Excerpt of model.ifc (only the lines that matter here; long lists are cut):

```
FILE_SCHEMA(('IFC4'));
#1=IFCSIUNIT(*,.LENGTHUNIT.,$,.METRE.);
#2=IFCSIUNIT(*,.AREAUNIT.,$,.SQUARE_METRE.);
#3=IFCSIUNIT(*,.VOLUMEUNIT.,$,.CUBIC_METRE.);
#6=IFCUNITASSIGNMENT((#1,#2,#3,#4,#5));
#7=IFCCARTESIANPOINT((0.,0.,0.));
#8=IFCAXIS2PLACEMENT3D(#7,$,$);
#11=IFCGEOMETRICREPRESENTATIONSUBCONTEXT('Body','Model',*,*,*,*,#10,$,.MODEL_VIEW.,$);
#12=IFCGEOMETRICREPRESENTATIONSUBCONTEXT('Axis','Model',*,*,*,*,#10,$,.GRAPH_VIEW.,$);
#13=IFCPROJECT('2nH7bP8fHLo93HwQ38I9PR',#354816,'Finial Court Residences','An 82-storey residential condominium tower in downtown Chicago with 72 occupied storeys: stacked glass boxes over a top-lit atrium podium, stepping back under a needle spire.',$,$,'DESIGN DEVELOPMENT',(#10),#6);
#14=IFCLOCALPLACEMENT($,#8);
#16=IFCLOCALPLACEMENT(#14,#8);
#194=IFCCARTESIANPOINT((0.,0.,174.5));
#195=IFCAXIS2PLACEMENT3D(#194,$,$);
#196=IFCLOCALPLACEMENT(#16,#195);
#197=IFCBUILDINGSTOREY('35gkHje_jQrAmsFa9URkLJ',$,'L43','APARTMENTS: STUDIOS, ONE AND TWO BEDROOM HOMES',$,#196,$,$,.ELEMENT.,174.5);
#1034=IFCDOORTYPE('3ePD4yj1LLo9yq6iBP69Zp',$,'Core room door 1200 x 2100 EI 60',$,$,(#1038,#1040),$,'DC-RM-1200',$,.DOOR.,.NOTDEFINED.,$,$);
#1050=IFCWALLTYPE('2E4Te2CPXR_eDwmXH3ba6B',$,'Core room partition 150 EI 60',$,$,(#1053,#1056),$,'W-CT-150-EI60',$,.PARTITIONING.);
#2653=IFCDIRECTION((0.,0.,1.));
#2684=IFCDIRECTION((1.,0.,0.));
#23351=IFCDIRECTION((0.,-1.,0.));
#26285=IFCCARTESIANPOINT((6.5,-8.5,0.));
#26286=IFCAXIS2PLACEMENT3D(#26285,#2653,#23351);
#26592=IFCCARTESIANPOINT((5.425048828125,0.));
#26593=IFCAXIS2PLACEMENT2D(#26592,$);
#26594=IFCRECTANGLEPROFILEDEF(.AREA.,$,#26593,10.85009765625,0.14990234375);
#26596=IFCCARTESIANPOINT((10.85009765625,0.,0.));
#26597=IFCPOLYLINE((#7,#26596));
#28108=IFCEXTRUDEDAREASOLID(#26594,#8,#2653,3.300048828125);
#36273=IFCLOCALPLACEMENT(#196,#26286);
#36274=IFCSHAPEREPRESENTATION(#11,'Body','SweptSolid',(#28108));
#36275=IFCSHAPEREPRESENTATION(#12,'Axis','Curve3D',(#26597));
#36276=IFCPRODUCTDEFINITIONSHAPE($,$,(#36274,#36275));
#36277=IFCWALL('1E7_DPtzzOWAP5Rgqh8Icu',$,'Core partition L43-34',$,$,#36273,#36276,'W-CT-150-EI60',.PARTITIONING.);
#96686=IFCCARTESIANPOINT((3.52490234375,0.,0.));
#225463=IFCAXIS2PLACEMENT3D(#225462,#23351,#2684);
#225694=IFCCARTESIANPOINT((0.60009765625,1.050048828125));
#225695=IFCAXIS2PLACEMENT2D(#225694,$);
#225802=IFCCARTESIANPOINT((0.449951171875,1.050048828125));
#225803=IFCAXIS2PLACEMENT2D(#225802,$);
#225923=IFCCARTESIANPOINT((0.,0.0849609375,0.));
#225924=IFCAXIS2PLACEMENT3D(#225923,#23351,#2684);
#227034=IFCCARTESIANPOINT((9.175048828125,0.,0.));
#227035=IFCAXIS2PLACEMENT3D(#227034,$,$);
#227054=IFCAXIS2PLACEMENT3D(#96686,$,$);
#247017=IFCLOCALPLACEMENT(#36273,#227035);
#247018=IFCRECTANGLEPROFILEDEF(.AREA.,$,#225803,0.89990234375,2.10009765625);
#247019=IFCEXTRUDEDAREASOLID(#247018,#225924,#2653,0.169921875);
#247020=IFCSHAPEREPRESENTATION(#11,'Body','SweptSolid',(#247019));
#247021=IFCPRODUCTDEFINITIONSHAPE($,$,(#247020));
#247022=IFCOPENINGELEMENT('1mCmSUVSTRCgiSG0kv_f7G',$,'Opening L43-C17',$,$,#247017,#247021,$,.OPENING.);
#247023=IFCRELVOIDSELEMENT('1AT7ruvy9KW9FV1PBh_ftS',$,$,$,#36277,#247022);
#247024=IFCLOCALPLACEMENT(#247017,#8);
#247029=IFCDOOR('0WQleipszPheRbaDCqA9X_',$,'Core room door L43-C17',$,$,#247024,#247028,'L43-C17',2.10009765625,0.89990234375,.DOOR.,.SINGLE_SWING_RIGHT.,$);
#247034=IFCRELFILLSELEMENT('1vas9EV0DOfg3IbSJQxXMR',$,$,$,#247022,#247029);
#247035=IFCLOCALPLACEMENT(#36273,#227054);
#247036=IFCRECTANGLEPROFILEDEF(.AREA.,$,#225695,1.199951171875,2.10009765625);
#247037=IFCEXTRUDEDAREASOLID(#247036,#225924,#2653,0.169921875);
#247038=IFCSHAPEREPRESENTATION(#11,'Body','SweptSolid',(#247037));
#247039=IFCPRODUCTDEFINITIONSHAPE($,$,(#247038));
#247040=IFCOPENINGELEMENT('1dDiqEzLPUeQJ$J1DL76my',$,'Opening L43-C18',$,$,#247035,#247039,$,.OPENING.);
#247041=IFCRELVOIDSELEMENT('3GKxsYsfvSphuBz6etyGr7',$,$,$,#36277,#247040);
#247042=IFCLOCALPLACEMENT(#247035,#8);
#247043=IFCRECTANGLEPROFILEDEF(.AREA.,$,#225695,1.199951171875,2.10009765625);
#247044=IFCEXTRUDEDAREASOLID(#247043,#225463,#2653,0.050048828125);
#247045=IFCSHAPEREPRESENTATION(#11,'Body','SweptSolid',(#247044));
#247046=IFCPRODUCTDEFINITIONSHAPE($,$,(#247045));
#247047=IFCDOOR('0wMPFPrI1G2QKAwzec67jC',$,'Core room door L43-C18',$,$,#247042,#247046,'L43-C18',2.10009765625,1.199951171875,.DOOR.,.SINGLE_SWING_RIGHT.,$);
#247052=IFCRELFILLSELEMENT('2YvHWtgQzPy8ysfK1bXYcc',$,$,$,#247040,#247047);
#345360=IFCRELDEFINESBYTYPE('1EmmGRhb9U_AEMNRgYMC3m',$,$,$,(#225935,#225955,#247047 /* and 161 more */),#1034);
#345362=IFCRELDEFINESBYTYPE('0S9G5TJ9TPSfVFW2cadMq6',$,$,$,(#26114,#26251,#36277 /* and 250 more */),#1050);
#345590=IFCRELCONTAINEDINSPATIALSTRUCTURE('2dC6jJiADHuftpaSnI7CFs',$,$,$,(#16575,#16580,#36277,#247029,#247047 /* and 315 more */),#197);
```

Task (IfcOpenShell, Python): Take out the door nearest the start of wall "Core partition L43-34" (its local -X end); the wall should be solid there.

```python
import ifcopenshell
import ifcopenshell.api.feature
import ifcopenshell.api.root
import ifcopenshell.geom
import ifcopenshell.util.shape

model = ifcopenshell.open("model.ifc")
settings = ifcopenshell.geom.settings()


def volume(element):
    """Net volume in cubic metres, openings subtracted."""
    shape = ifcopenshell.geom.create_shape(settings, element)
    return ifcopenshell.util.shape.get_volume(shape.geometry)


door = model.by_guid("0wMPFPrI1G2QKAwzec67jC")
opening = door.FillsVoids[0].RelatingOpeningElement
wall = opening.VoidsElements[0].RelatingBuildingElement
before = volume(wall)

ifcopenshell.api.root.remove_product(model, product=door)
ifcopenshell.api.feature.remove_feature(model, feature=opening)

after = volume(wall)

print(f"wall volume {before:.3f} -> {after:.3f} m3")

model.write("model-out.ifc")
```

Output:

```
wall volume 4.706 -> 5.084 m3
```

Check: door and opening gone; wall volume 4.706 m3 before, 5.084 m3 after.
